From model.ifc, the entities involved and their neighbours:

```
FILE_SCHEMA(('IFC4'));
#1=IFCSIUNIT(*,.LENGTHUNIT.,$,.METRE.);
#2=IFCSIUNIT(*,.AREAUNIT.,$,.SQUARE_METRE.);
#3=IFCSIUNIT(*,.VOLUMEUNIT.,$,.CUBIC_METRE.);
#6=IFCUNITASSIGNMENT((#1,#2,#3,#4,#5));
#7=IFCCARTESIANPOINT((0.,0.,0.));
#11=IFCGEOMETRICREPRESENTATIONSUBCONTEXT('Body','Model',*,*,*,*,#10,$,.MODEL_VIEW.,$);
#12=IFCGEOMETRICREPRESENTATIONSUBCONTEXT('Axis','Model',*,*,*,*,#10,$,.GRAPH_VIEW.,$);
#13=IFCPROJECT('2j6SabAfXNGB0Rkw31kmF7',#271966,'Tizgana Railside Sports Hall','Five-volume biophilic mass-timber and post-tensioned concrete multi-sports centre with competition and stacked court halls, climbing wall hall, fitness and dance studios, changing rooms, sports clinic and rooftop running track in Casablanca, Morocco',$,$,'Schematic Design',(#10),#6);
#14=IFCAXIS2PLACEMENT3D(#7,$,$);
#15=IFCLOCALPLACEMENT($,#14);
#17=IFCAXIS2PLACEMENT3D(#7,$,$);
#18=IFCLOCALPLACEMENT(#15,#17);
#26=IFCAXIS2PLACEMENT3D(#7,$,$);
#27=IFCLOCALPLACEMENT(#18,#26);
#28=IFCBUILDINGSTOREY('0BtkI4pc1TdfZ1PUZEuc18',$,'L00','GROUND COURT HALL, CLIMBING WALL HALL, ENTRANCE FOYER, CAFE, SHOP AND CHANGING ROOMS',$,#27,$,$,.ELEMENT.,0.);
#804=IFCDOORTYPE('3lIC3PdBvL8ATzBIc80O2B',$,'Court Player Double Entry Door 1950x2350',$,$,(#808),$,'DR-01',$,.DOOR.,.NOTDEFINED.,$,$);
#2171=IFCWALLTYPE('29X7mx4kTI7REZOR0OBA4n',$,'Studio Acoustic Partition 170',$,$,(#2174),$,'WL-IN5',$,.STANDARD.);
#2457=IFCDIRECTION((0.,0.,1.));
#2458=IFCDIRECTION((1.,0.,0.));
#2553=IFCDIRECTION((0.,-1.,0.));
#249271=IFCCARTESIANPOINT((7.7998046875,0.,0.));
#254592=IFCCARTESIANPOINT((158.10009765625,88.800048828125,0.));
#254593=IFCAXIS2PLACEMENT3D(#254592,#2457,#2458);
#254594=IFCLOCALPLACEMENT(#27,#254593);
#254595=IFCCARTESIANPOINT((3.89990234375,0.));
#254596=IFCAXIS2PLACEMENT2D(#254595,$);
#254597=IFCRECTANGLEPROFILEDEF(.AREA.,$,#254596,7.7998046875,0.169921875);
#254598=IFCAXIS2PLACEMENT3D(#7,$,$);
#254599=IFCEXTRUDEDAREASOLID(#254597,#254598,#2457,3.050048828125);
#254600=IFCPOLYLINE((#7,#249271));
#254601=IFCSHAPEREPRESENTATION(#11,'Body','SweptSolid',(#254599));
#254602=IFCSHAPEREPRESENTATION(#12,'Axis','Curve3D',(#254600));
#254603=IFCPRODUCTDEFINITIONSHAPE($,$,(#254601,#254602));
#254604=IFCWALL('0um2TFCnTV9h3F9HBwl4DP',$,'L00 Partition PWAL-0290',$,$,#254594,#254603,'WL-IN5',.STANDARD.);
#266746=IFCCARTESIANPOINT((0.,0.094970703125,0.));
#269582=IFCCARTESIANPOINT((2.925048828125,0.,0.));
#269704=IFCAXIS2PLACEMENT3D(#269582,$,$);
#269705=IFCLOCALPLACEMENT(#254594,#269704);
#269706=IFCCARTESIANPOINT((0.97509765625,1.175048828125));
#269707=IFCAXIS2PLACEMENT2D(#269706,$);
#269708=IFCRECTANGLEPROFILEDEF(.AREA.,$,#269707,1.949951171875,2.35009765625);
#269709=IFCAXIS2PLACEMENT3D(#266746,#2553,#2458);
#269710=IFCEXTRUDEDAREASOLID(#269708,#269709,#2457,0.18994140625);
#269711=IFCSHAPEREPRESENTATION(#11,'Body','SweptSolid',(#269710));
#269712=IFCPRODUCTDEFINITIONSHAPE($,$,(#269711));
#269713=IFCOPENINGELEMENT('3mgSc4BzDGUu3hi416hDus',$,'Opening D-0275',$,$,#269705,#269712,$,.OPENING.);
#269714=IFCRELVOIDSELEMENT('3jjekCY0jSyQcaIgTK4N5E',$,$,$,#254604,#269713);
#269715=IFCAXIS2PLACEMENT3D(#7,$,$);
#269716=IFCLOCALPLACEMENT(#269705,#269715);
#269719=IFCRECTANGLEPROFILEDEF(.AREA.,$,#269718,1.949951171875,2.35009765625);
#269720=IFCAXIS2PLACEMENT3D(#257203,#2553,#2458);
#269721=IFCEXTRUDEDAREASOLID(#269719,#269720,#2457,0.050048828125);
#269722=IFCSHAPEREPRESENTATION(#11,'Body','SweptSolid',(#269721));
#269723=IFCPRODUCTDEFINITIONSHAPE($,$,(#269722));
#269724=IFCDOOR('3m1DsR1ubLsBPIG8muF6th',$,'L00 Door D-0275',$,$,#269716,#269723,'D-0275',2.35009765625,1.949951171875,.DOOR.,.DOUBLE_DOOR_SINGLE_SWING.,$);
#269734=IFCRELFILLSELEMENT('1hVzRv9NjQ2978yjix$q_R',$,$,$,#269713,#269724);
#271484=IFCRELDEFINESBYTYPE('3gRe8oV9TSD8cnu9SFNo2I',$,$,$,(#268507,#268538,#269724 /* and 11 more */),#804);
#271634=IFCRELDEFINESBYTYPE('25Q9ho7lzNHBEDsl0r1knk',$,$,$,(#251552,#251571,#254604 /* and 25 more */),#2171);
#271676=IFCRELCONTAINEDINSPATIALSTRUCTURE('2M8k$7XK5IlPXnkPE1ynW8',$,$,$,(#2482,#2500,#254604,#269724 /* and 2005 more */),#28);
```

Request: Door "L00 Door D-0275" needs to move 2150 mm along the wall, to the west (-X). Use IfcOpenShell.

```python
import ifcopenshell
import ifcopenshell.api.geometry
import ifcopenshell.util.placement
import ifcopenshell.util.unit

model = ifcopenshell.open("model.ifc")
unit_scale = ifcopenshell.util.unit.calculate_unit_scale(model)

door = model.by_id(269724)
opening = door.FillsVoids[0].RelatingOpeningElement
wall = opening.VoidsElements[0].RelatingBuildingElement

wall_matrix = ifcopenshell.util.placement.get_local_placement(wall.ObjectPlacement)
shift = wall_matrix[:3, 0] * -2.15 / unit_scale
before = ifcopenshell.util.placement.get_local_placement(door.ObjectPlacement)[:3, 3].copy()

# The door is placed relative to its opening, so it follows when the opening moves.
matrix = ifcopenshell.util.placement.get_local_placement(opening.ObjectPlacement)
matrix[:3, 3] += shift
ifcopenshell.api.geometry.edit_object_placement(
    model, product=opening, matrix=matrix, is_si=False, should_transform_children=True
)

after = ifcopenshell.util.placement.get_local_placement(door.ObjectPlacement)[:3, 3]
print("door moved by", (after - before).round(3) + 0.0)

model.write("model_v2.ifc")
```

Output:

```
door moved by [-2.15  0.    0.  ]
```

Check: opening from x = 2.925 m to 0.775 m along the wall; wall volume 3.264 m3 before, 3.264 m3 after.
